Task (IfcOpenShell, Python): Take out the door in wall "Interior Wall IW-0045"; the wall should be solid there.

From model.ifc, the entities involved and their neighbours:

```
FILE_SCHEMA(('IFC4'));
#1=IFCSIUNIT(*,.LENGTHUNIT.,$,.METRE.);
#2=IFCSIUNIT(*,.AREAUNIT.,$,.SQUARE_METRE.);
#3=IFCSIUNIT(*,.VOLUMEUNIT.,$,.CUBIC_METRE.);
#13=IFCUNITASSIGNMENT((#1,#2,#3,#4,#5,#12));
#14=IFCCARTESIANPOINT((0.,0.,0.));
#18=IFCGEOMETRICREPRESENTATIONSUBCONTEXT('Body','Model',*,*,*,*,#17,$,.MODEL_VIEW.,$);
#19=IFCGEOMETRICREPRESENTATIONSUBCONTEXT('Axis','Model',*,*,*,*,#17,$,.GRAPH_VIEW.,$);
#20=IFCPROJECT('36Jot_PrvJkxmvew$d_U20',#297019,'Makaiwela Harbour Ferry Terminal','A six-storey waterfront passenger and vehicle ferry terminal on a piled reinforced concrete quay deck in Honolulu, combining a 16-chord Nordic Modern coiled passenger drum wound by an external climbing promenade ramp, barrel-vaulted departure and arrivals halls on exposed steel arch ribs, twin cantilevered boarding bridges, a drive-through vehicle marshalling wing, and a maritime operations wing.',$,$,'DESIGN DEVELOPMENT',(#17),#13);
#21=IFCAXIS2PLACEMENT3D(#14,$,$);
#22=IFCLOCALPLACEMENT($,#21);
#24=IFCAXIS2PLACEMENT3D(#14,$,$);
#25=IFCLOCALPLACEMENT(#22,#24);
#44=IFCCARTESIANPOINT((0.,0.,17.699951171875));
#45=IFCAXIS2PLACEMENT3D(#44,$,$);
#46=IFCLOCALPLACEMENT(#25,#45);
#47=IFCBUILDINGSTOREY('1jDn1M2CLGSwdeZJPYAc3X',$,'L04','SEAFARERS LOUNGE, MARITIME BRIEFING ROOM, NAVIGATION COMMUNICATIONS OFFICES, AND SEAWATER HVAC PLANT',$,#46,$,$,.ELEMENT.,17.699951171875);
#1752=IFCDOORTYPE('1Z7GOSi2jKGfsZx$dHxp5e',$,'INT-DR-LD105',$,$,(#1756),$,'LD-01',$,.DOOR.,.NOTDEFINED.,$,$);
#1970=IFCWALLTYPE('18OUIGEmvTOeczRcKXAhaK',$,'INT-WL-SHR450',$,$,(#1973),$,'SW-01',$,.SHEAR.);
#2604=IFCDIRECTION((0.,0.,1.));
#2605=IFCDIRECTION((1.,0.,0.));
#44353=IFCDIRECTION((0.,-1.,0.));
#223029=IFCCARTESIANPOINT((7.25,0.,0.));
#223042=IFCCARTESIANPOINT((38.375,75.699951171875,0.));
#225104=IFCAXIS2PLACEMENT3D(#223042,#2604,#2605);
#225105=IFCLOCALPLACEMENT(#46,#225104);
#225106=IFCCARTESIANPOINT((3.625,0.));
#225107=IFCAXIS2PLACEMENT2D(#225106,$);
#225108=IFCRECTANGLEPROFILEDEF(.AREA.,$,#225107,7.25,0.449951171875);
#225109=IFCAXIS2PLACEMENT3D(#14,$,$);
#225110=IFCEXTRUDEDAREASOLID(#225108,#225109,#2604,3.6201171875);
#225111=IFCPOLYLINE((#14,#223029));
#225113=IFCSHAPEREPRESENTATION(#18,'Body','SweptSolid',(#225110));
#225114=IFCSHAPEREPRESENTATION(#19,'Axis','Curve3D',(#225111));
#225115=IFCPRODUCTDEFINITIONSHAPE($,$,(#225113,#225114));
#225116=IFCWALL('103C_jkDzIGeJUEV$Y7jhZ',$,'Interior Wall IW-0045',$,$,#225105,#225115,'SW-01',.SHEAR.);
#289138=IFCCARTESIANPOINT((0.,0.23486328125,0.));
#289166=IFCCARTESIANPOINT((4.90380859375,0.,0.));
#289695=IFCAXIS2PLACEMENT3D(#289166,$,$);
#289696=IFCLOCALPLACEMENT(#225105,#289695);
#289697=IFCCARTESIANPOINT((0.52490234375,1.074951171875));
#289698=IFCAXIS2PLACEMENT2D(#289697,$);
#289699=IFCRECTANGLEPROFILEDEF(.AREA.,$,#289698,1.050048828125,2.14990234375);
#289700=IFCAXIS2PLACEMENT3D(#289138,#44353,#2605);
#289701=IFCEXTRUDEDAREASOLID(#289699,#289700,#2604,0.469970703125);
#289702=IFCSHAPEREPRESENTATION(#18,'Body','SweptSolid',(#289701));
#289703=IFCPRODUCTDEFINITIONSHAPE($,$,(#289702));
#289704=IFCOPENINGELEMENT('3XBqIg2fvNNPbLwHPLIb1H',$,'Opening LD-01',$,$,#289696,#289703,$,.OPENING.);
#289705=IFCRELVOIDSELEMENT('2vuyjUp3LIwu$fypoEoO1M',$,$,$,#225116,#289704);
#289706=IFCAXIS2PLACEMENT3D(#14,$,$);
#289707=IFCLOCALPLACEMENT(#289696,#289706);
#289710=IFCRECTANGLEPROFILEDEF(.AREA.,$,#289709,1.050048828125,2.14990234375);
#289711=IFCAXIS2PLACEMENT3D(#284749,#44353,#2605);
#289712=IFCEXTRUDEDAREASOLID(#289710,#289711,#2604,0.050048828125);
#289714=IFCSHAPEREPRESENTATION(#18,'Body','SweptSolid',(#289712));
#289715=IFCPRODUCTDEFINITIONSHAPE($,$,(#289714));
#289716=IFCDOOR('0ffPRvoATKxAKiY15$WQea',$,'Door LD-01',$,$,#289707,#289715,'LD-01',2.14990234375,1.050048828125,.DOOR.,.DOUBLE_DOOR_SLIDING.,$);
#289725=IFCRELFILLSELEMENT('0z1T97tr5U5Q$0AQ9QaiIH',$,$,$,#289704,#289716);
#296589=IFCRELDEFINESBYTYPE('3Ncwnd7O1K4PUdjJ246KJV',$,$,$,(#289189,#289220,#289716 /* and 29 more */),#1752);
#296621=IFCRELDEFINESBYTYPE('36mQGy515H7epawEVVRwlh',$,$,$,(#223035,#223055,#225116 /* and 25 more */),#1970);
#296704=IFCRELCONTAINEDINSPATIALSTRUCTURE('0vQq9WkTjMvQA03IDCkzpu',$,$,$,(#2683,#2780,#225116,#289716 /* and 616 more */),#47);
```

```python
import ifcopenshell
import ifcopenshell.api.feature
import ifcopenshell.api.root
import ifcopenshell.geom
import ifcopenshell.util.shape

model = ifcopenshell.open("model.ifc")
settings = ifcopenshell.geom.settings()


def volume(element):
    """Net volume in cubic metres, openings subtracted."""
    shape = ifcopenshell.geom.create_shape(settings, element)
    return ifcopenshell.util.shape.get_volume(shape.geometry)


door = model.by_id(289716)
opening = door.FillsVoids[0].RelatingOpeningElement
wall = opening.VoidsElements[0].RelatingBuildingElement
before = volume(wall)

ifcopenshell.api.root.remove_product(model, product=door)
ifcopenshell.api.feature.remove_feature(model, feature=opening)

after = volume(wall)

print(f"wall volume {before:.3f} -> {after:.3f} m3")

model.write("model_updated.ifc")
```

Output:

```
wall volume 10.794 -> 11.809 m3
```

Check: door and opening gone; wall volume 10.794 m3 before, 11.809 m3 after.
